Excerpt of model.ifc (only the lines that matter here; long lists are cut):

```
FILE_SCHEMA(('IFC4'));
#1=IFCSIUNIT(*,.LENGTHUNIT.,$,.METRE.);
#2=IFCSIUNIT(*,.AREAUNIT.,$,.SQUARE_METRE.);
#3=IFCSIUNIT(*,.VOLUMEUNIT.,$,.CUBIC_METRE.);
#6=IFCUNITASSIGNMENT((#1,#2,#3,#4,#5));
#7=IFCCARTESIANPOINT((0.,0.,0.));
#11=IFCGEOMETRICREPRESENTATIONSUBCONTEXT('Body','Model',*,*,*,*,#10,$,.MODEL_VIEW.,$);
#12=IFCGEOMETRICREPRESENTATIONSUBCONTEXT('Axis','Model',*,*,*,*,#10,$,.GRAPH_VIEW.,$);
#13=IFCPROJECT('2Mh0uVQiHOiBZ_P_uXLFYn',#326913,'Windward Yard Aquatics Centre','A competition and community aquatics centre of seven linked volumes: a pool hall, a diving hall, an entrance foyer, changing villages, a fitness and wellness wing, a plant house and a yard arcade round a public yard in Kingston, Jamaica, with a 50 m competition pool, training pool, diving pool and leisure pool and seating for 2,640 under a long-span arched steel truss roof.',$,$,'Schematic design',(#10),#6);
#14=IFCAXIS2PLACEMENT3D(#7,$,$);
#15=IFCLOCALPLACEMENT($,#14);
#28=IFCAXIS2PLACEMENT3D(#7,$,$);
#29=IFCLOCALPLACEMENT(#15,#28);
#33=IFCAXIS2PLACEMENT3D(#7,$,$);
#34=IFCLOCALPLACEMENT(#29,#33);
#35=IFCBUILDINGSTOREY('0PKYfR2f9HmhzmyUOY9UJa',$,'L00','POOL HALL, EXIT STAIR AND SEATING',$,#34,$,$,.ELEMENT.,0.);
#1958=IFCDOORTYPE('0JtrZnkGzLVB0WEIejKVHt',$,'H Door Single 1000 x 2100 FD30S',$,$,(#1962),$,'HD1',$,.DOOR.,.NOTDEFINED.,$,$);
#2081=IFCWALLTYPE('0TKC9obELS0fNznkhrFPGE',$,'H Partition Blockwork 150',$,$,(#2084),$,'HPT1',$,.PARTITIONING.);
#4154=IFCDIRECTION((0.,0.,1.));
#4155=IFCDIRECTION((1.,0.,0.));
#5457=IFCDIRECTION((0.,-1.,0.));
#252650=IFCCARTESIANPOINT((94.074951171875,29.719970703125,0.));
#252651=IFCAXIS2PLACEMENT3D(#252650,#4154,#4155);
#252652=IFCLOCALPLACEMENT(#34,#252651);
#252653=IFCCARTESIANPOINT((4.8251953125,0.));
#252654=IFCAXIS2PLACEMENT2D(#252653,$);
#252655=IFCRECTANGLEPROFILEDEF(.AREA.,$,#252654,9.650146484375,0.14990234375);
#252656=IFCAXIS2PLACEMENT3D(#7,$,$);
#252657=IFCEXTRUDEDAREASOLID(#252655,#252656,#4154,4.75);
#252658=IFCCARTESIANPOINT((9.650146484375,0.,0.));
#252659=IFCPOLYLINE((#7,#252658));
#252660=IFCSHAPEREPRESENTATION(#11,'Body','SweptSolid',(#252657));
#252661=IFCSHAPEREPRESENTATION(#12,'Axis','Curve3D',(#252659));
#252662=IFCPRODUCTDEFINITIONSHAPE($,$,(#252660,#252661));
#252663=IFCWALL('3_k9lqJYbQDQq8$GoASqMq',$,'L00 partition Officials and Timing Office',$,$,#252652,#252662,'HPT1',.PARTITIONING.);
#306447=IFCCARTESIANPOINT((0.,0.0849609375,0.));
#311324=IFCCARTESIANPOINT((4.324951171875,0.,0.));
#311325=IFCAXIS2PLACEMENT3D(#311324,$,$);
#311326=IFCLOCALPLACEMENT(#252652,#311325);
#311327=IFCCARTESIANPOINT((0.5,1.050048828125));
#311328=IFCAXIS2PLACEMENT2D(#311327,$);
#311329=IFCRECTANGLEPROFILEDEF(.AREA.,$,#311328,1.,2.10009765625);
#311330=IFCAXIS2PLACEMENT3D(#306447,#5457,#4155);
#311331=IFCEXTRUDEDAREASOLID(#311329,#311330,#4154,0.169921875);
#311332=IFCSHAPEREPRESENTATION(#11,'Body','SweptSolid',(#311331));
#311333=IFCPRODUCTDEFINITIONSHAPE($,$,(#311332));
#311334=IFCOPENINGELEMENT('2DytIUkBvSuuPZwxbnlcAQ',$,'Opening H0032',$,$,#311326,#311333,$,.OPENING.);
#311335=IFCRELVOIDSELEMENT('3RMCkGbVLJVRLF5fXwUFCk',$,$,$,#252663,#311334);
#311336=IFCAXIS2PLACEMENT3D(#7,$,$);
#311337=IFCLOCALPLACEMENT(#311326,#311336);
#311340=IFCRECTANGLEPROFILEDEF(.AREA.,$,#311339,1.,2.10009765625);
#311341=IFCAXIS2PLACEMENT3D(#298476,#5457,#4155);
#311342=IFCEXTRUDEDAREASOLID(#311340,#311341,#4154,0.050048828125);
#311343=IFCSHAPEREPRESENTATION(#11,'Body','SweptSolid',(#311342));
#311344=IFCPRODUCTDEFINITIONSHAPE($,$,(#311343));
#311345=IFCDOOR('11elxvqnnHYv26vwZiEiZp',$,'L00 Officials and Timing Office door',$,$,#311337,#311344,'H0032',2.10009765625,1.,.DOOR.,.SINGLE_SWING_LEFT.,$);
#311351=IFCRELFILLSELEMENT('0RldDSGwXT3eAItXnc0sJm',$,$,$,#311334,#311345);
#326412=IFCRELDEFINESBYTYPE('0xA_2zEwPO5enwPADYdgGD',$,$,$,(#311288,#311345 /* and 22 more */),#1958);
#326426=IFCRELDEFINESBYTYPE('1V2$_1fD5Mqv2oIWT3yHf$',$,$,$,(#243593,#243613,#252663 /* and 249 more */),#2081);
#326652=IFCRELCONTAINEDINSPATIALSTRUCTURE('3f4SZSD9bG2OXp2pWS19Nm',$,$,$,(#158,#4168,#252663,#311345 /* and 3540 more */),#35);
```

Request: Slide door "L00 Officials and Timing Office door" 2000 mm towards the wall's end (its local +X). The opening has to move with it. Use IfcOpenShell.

```python
import ifcopenshell
import ifcopenshell.api.geometry
import ifcopenshell.util.placement
import ifcopenshell.util.unit

model = ifcopenshell.open("model.ifc")
unit_scale = ifcopenshell.util.unit.calculate_unit_scale(model)

door = model.by_guid("11elxvqnnHYv26vwZiEiZp")
opening = door.FillsVoids[0].RelatingOpeningElement
wall = opening.VoidsElements[0].RelatingBuildingElement

wall_matrix = ifcopenshell.util.placement.get_local_placement(wall.ObjectPlacement)
shift = wall_matrix[:3, 0] * 2 / unit_scale
before = ifcopenshell.util.placement.get_local_placement(door.ObjectPlacement)[:3, 3].copy()

# The door is placed relative to its opening, so it follows when the opening moves.
matrix = ifcopenshell.util.placement.get_local_placement(opening.ObjectPlacement)
matrix[:3, 3] += shift
ifcopenshell.api.geometry.edit_object_placement(
    model, product=opening, matrix=matrix, is_si=False, should_transform_children=True
)

after = ifcopenshell.util.placement.get_local_placement(door.ObjectPlacement)[:3, 3]
print("door moved by", (after - before).round(3) + 0.0)

model.write("model_v2.ifc")
```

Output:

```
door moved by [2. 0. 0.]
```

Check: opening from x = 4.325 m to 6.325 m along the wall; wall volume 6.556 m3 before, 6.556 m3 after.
